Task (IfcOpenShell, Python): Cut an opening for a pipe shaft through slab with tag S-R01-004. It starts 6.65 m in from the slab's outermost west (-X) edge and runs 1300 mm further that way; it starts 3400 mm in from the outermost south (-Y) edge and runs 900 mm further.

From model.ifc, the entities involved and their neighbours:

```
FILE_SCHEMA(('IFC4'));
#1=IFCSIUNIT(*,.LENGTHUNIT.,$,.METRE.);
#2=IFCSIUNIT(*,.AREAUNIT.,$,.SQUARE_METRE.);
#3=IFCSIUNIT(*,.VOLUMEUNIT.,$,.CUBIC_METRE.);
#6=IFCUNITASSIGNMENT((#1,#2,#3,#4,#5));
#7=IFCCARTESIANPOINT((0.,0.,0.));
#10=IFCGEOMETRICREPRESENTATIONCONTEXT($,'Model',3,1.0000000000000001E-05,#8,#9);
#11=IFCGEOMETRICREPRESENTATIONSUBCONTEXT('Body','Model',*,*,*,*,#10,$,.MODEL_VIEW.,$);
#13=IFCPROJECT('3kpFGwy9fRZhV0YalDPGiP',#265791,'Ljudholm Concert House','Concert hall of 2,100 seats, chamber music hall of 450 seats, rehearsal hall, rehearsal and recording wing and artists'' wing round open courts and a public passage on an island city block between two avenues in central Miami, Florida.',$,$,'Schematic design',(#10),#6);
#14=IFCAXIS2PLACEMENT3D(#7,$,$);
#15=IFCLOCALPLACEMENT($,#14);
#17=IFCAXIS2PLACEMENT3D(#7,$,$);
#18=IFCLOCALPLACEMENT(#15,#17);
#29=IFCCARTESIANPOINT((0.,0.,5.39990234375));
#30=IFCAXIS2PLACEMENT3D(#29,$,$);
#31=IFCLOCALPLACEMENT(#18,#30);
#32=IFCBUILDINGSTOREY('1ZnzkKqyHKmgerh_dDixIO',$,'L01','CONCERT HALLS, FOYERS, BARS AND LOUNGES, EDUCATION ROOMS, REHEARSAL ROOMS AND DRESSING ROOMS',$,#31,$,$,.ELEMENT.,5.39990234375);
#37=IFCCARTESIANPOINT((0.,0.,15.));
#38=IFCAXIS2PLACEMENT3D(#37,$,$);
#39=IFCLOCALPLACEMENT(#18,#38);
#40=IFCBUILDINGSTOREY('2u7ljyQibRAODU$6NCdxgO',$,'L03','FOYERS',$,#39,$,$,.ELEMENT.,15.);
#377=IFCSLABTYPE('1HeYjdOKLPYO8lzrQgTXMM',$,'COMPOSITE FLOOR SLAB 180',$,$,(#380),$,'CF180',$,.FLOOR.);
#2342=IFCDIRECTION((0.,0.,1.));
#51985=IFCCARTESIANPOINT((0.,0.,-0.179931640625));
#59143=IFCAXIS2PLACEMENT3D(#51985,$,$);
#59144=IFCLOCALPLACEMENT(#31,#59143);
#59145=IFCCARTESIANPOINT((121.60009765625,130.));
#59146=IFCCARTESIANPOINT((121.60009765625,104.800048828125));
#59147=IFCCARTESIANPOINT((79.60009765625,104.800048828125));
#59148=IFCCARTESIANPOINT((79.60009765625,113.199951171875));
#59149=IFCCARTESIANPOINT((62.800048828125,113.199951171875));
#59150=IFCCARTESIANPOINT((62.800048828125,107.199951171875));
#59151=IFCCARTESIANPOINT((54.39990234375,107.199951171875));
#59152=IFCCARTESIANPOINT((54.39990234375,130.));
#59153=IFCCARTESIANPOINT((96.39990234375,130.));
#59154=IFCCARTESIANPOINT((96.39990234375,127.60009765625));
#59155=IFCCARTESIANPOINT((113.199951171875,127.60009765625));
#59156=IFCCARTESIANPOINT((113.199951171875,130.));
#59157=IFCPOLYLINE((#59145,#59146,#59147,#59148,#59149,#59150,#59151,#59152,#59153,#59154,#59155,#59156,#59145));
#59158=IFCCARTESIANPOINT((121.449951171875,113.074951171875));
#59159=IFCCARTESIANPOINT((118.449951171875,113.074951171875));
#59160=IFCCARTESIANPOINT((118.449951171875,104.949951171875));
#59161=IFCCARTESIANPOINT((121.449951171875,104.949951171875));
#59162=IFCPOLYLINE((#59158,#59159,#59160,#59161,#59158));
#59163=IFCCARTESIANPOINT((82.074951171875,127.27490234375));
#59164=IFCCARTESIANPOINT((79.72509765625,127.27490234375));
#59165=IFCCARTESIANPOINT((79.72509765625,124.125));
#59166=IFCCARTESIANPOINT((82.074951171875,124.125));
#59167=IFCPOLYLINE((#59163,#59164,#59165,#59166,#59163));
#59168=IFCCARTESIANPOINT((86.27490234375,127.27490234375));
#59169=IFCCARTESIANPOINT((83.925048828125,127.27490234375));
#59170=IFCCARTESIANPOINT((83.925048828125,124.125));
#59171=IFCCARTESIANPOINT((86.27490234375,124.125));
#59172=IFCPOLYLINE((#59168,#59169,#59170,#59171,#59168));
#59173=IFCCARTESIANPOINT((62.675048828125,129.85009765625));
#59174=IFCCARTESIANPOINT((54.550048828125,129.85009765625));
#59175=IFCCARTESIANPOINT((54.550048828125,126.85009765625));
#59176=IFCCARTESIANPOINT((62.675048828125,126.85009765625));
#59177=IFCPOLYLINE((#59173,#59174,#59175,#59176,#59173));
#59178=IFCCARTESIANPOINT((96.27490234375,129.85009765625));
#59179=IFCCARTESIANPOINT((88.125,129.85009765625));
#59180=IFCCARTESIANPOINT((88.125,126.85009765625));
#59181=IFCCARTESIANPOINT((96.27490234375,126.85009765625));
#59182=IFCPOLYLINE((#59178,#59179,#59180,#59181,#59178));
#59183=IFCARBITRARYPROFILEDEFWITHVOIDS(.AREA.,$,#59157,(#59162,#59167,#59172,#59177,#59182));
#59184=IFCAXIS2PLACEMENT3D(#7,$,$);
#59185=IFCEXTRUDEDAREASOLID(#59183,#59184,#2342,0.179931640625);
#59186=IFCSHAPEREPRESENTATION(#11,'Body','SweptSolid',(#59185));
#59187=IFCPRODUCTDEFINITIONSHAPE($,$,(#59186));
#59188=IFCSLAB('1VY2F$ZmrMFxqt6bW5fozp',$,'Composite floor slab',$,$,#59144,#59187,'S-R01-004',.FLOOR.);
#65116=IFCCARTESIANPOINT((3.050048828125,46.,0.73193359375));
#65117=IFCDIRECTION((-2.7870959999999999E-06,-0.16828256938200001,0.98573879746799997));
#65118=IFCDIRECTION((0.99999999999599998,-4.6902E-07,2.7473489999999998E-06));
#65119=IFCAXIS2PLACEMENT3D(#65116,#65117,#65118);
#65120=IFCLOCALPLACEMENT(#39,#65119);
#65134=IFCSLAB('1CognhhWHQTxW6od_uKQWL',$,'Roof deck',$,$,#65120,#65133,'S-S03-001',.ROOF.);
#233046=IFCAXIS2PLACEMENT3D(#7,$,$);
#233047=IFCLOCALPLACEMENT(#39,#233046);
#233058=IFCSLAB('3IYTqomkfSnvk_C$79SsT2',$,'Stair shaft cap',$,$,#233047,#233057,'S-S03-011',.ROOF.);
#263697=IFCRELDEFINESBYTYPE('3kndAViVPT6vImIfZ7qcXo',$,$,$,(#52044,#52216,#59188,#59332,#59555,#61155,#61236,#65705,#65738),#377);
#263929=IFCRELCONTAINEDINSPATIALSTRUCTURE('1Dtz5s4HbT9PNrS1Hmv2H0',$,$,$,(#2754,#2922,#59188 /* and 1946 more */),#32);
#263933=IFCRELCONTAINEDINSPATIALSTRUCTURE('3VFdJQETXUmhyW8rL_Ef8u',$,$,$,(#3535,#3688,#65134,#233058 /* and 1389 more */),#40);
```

```python
import numpy as np
import ifcopenshell
import ifcopenshell.api.feature
import ifcopenshell.api.geometry
import ifcopenshell.api.root
import ifcopenshell.geom
import ifcopenshell.util.placement
import ifcopenshell.util.representation
import ifcopenshell.util.shape
import ifcopenshell.util.unit

model = ifcopenshell.open("model.ifc")
unit_scale = ifcopenshell.util.unit.calculate_unit_scale(model)
settings = ifcopenshell.geom.settings()


def volume(element):
    """Net volume in cubic metres, openings subtracted."""
    shape = ifcopenshell.geom.create_shape(settings, element)
    return ifcopenshell.util.shape.get_volume(shape.geometry)


slab = model.by_id(59188)
before = volume(slab)

# Extent in the slab's own axes, in metres. The edges named are its -X and -Y sides.
slab_shape = ifcopenshell.geom.create_shape(settings, slab)
vertices = ifcopenshell.util.shape.get_vertices(slab_shape.geometry)
x_min, y_min, bottom = vertices.min(axis=0)
top = vertices[:, 2].max()

opening = ifcopenshell.api.root.create_entity(model, ifc_class="IfcOpeningElement", name="Pipe shaft opening", predefined_type="OPENING")
context = ifcopenshell.util.representation.get_context(model, "Model", "Body", "MODEL_VIEW")
width, depth = 1.3, 0.9
outline = [(0.0, 0.0), (width, 0.0), (width, depth), (0.0, depth), (0.0, 0.0)]
# Overshoot both faces by 50 mm so the cut is clean.
shape = ifcopenshell.api.geometry.add_slab_representation(
    model, context=context, depth=top - bottom + 0.1, polyline=outline
)
ifcopenshell.api.geometry.assign_representation(model, product=opening, representation=shape)

matrix = ifcopenshell.util.placement.get_local_placement(slab.ObjectPlacement)
matrix[:, 3] = matrix @ np.append(np.array([x_min + 6.65, y_min + 3.4, bottom - 0.05]) / unit_scale, 1.0)
ifcopenshell.api.geometry.edit_object_placement(model, product=opening, matrix=matrix, is_si=False)
ifcopenshell.api.feature.add_feature(model, feature=opening, element=slab)

after = volume(slab)

print(f"slab volume {before:.3f} -> {after:.3f} m3")

model.write("model-out.ifc")
```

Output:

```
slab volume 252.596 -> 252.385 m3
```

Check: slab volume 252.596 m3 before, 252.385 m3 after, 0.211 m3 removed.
